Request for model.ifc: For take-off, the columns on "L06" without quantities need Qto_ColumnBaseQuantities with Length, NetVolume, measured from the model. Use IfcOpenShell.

First a look at what the model holds.

```python
import ifcopenshell
import ifcopenshell.util.element
import ifcopenshell.util.unit

model = ifcopenshell.open("model.ifc")
print(model.schema)
for unit_type in ("LENGTHUNIT", "AREAUNIT", "VOLUMEUNIT"):
    print(unit_type, ifcopenshell.util.unit.calculate_unit_scale(model, unit_type))
storey = next(s for s in model.by_type("IfcBuildingStorey") if s.Name == "L06")
columns = [e for e in ifcopenshell.util.element.get_decomposition(storey) if e.is_a("IfcColumn")]
for e in sorted(columns, key=lambda e: e.id()):
    print(e.id(), e.is_a(), e.Name, list(ifcopenshell.util.element.get_psets(e, qtos_only=True)), sep=" | ")
```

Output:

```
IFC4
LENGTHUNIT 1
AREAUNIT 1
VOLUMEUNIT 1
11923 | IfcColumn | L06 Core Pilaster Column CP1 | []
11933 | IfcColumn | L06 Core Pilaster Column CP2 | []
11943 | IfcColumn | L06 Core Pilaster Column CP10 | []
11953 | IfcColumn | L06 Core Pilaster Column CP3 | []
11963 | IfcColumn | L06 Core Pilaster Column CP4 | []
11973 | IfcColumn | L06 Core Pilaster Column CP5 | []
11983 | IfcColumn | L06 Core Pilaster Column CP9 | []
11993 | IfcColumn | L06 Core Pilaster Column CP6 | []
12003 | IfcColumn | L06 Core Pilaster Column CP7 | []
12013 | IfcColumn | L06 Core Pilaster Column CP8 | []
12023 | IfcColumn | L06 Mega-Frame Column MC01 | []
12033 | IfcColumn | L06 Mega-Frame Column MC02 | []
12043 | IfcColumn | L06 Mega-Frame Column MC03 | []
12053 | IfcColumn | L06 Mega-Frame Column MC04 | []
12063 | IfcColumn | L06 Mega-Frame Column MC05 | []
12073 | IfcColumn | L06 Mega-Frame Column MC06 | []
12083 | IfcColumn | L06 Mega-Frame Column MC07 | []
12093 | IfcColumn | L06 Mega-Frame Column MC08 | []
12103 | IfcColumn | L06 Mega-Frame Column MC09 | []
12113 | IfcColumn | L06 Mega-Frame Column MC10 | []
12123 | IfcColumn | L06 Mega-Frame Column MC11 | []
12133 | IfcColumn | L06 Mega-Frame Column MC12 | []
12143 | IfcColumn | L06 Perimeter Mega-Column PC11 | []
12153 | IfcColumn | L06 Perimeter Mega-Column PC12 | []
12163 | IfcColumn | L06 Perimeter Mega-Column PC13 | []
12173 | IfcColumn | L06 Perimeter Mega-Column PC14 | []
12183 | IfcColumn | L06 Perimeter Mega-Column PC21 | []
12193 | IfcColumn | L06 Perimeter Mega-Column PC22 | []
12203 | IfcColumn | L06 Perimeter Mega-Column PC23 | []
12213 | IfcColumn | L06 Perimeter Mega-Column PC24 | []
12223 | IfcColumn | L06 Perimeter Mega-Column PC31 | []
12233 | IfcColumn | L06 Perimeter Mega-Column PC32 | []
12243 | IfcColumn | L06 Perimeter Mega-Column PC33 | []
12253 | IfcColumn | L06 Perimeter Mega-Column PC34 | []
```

```python
import ifcopenshell
import ifcopenshell.api.pset
import ifcopenshell.geom
import ifcopenshell.util.element
import ifcopenshell.util.shape
import ifcopenshell.util.unit

model = ifcopenshell.open("model.ifc")
unit_scale = ifcopenshell.util.unit.calculate_unit_scale(model)
volume_scale = ifcopenshell.util.unit.calculate_unit_scale(model, "VOLUMEUNIT")
settings = ifcopenshell.geom.settings()

storey = next(s for s in model.by_type("IfcBuildingStorey") if s.Name == "L06")
columns = [e for e in ifcopenshell.util.element.get_decomposition(storey) if e.is_a("IfcColumn")]

for e in sorted(columns, key=lambda e: e.id()):
    if ifcopenshell.util.element.get_psets(e, qtos_only=True, should_inherit=False):
        continue
    # Geometry comes back in metres, in the element's own axes.
    shape = ifcopenshell.geom.create_shape(settings, e)
    values = {
        "Length": ifcopenshell.util.shape.get_z(shape.geometry) / unit_scale,
        "NetVolume": ifcopenshell.util.shape.get_volume(shape.geometry) / volume_scale,
    }
    qto = ifcopenshell.api.pset.add_qto(model, product=e, name="Qto_ColumnBaseQuantities")
    ifcopenshell.api.pset.edit_qto(model, qto=qto, properties=values)
    print(e.id(), {k: round(v, 3) for k, v in values.items()})

model.write("model_updated.ifc")
```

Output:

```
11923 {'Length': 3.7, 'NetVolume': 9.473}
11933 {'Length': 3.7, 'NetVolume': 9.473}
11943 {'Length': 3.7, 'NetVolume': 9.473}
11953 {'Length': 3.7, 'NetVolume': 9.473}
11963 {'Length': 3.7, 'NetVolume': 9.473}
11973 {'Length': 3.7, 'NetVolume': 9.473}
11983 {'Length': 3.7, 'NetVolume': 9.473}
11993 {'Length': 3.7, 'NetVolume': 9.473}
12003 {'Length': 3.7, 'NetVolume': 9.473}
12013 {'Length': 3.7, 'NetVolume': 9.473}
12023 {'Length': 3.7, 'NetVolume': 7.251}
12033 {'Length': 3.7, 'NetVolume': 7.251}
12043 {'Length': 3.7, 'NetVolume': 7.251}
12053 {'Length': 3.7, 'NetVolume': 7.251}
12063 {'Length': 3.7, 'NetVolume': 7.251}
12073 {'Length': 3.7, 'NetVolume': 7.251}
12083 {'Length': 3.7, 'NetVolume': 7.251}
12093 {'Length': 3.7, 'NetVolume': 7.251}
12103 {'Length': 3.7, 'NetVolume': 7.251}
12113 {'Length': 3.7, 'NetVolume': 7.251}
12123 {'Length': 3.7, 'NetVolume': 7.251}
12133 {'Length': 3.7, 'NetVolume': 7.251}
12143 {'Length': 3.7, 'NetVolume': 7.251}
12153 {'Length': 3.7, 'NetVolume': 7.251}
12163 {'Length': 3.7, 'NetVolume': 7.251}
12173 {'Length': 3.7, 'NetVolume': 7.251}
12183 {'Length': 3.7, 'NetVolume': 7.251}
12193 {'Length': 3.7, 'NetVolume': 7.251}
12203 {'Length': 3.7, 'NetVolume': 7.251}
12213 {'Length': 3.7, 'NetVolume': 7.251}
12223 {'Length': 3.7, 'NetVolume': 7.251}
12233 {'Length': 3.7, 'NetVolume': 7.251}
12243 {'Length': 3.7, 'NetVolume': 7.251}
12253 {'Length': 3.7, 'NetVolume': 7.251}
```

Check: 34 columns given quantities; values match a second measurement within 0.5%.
